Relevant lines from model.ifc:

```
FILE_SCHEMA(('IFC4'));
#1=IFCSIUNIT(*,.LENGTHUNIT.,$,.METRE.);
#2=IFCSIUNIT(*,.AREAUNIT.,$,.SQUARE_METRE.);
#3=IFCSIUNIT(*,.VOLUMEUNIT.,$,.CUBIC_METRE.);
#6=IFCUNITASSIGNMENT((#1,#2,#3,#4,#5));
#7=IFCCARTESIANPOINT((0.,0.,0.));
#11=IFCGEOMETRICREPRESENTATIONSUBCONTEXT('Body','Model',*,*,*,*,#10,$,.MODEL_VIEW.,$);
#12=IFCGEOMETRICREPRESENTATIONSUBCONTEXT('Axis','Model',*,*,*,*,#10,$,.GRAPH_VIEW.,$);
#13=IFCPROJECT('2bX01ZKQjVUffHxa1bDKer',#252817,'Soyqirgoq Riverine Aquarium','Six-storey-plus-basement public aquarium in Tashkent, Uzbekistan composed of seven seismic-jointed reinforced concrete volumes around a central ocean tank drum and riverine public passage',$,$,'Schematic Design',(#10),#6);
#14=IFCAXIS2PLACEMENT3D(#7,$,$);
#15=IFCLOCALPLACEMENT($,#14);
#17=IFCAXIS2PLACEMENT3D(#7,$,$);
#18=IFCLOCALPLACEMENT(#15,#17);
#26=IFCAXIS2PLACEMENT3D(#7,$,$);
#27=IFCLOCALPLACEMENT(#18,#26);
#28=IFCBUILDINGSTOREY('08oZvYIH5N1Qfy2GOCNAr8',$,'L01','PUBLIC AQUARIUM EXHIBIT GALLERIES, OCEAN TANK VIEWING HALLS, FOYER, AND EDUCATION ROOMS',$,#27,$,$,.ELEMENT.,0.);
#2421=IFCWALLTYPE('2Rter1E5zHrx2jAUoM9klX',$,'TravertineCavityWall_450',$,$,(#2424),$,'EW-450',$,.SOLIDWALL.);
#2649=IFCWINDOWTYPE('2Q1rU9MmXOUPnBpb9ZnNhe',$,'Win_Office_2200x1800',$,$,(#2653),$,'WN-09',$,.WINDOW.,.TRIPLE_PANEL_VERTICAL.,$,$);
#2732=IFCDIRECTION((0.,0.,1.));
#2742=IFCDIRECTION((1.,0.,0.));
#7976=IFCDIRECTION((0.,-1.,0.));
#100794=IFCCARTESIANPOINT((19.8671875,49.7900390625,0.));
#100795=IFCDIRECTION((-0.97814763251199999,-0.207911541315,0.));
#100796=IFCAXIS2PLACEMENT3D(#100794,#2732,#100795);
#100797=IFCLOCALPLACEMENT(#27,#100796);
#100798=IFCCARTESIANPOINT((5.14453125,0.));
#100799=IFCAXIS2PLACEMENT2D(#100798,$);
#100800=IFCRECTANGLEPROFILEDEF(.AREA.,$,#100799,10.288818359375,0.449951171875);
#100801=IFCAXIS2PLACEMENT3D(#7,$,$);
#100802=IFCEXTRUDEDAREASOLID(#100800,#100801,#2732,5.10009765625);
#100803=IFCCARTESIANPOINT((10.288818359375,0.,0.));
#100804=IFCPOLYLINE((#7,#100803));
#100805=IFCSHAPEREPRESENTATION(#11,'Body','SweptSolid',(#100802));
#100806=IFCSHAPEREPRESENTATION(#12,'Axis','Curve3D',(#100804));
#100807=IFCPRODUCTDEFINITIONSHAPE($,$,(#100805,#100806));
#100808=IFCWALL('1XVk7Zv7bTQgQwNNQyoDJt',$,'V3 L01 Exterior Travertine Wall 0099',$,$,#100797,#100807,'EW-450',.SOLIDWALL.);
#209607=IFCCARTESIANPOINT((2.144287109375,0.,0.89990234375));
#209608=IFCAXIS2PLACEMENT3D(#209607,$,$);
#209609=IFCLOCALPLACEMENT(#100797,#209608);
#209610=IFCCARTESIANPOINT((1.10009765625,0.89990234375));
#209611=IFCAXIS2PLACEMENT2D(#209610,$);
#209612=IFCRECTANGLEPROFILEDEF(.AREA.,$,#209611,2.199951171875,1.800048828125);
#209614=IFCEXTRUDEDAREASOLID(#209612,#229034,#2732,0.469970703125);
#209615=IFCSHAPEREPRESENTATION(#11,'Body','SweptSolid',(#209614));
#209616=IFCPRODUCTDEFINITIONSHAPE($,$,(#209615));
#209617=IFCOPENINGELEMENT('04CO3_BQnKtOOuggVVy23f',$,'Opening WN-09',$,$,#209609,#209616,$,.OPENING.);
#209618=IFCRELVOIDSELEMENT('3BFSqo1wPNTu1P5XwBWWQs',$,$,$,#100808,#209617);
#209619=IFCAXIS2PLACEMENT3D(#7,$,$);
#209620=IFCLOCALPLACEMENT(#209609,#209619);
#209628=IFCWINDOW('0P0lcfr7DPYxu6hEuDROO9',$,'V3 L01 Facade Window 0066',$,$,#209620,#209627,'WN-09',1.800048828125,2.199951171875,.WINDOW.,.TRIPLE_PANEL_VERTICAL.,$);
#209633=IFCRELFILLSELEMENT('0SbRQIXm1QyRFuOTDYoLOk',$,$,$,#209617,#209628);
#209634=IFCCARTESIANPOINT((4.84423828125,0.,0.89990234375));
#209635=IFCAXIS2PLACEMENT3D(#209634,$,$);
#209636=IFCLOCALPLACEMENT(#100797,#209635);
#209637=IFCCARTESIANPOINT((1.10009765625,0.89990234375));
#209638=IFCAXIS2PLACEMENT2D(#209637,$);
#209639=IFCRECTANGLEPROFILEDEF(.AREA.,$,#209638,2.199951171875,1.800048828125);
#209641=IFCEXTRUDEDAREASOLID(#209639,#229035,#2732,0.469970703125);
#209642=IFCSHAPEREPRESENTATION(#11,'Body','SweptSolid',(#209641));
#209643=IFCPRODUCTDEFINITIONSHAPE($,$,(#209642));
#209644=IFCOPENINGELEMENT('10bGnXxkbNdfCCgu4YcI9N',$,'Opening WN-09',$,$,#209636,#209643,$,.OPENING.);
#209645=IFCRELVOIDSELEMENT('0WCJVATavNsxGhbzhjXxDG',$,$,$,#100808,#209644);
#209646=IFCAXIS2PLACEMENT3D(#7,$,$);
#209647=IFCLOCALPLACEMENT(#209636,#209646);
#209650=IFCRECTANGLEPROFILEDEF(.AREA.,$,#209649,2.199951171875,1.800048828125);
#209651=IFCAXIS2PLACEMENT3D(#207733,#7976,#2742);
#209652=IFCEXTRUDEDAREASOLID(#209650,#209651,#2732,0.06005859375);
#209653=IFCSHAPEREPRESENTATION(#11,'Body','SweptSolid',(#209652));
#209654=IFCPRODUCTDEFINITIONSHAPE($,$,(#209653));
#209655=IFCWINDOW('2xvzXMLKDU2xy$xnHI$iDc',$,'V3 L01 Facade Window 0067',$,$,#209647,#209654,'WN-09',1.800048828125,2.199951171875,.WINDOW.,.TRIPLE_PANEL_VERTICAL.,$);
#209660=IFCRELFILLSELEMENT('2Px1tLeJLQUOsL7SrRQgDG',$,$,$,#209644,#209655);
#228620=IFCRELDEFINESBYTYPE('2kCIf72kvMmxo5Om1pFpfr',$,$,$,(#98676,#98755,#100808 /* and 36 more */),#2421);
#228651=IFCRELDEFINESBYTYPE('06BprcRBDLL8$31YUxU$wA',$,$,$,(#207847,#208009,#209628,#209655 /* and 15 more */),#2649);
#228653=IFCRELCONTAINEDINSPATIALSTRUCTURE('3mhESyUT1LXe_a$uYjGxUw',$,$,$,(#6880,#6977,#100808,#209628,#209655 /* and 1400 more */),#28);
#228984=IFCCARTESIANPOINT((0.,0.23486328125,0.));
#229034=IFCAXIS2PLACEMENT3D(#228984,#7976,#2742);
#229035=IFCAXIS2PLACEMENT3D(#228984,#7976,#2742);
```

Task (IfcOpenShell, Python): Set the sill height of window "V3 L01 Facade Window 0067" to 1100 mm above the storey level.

```python
import numpy as np
import ifcopenshell
import ifcopenshell.api.geometry
import ifcopenshell.geom
import ifcopenshell.util.element
import ifcopenshell.util.placement
import ifcopenshell.util.shape
import ifcopenshell.util.unit

model = ifcopenshell.open("model.ifc")
unit_scale = ifcopenshell.util.unit.calculate_unit_scale(model)

window = model.by_guid("2xvzXMLKDU2xy$xnHI$iDc")
opening = window.FillsVoids[0].RelatingOpeningElement
storey = ifcopenshell.util.element.get_container(window, ifc_class="IfcBuildingStorey")
level = ifcopenshell.util.placement.get_local_placement(storey.ObjectPlacement)[2, 3]

# The opening's origin need not be at the sill, so measure its lowest point.
shape = ifcopenshell.geom.create_shape(ifcopenshell.geom.settings(), opening)
bottom = ifcopenshell.util.shape.get_shape_bottom_elevation(shape, shape.geometry) / unit_scale
dz = level + 1.1 - bottom

shift = np.array([0.0, 0.0, dz])
# The window is placed relative to its opening, so it follows when the opening moves.
matrix = ifcopenshell.util.placement.get_local_placement(opening.ObjectPlacement)
matrix[:3, 3] += shift
ifcopenshell.api.geometry.edit_object_placement(
    model, product=opening, matrix=matrix, is_si=False, should_transform_children=True
)

print(f"moved by {dz * unit_scale:+.3f} m")

model.write("model_edited.ifc")
```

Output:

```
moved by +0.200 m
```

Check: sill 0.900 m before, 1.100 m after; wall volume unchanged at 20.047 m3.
